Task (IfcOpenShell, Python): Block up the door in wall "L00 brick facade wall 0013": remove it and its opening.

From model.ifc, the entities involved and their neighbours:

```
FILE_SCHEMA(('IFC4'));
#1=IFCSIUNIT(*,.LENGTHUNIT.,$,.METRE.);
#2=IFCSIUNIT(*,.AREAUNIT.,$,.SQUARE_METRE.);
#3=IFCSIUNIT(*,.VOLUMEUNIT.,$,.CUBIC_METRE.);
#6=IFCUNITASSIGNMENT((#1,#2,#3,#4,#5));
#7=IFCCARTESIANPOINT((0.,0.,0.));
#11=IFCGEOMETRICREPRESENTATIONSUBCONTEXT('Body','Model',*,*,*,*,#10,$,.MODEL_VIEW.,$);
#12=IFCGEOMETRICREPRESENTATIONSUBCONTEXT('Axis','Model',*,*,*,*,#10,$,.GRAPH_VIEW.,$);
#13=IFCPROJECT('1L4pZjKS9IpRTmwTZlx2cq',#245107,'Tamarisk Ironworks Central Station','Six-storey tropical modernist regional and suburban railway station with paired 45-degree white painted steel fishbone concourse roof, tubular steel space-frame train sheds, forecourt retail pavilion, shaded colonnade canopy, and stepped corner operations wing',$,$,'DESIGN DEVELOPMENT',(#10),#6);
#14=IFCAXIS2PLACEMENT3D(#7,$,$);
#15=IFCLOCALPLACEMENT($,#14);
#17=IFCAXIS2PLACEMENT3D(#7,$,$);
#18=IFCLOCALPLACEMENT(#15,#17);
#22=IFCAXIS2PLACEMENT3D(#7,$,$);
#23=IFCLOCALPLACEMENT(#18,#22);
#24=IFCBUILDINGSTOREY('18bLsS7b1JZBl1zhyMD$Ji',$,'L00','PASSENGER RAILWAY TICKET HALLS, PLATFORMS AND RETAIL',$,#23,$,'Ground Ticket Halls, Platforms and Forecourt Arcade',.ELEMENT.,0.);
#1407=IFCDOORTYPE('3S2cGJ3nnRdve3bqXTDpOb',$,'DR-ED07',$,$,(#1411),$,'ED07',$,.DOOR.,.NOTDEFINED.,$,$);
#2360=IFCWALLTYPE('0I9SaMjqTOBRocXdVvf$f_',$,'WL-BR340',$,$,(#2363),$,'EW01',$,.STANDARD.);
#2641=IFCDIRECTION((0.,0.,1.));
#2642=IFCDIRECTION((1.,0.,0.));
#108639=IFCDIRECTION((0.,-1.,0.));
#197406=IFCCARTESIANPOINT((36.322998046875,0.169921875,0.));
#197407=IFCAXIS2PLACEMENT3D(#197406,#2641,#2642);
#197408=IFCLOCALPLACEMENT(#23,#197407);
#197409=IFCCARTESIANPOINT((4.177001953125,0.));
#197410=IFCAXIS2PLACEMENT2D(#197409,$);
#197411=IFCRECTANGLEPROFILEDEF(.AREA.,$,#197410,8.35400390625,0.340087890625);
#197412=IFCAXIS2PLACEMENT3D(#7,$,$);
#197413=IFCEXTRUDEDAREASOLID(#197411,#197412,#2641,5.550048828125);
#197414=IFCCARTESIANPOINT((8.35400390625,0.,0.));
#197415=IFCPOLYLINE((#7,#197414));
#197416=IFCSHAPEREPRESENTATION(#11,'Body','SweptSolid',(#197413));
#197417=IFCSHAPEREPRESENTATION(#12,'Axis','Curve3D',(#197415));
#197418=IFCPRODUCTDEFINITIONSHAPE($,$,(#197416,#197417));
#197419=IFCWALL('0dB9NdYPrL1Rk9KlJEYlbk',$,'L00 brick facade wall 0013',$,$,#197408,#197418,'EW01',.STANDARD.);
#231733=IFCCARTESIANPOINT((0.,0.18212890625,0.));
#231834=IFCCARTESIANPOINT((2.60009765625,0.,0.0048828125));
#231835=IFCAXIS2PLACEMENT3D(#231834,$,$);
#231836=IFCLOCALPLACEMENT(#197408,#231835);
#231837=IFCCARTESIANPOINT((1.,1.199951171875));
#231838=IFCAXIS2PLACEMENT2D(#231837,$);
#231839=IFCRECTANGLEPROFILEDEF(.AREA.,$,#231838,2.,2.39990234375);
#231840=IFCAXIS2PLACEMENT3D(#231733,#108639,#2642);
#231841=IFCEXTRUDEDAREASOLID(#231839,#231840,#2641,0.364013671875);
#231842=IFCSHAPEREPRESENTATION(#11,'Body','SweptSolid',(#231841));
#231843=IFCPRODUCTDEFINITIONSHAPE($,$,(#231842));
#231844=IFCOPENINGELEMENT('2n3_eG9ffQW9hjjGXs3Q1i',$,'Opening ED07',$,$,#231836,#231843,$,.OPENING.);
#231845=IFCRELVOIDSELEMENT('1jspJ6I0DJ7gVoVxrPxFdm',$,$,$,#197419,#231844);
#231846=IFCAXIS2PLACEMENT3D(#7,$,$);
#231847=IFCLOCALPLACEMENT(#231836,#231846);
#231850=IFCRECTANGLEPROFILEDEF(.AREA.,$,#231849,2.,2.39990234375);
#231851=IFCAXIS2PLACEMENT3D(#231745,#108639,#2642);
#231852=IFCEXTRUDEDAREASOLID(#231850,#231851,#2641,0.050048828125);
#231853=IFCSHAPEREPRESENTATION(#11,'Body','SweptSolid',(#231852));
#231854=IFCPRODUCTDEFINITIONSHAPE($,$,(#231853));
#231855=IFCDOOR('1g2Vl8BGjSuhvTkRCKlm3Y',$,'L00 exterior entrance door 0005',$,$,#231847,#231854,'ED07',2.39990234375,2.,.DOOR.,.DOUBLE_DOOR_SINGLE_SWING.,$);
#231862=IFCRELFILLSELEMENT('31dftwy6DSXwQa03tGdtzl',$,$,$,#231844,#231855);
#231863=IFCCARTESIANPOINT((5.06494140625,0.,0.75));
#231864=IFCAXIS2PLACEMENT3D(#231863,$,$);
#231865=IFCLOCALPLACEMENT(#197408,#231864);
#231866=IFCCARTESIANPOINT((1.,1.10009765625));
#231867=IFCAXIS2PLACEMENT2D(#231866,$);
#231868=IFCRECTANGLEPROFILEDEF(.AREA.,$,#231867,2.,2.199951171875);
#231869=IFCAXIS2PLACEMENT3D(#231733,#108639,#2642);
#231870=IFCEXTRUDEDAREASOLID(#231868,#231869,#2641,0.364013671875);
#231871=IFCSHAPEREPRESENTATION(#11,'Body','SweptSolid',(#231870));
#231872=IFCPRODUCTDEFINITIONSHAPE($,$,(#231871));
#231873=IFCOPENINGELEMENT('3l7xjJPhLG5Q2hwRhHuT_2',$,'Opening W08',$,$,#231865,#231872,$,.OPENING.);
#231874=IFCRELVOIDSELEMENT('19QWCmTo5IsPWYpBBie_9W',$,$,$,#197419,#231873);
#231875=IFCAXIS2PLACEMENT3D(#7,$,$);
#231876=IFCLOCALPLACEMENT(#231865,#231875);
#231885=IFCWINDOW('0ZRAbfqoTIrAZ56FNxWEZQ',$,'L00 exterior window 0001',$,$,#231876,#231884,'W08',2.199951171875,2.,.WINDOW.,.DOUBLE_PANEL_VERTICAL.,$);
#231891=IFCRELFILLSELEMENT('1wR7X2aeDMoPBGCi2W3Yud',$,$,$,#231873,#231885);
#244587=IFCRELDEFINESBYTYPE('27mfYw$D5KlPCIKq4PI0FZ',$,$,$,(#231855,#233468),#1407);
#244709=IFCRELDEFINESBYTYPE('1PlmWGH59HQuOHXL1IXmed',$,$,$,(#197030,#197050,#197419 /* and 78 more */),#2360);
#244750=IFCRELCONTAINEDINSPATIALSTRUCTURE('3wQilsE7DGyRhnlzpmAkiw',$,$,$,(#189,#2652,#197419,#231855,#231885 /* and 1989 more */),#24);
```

```python
import ifcopenshell
import ifcopenshell.api.feature
import ifcopenshell.api.root
import ifcopenshell.geom
import ifcopenshell.util.shape

model = ifcopenshell.open("model.ifc")
settings = ifcopenshell.geom.settings()


def volume(element):
    """Net volume in cubic metres, openings subtracted."""
    shape = ifcopenshell.geom.create_shape(settings, element)
    return ifcopenshell.util.shape.get_volume(shape.geometry)


door = model.by_id(231855)
opening = door.FillsVoids[0].RelatingOpeningElement
wall = opening.VoidsElements[0].RelatingBuildingElement
before = volume(wall)

ifcopenshell.api.root.remove_product(model, product=door)
ifcopenshell.api.feature.remove_feature(model, feature=opening)

after = volume(wall)

print(f"wall volume {before:.3f} -> {after:.3f} m3")

model.write("model_updated.ifc")
```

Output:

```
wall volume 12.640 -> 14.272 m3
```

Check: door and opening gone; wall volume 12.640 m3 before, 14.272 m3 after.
